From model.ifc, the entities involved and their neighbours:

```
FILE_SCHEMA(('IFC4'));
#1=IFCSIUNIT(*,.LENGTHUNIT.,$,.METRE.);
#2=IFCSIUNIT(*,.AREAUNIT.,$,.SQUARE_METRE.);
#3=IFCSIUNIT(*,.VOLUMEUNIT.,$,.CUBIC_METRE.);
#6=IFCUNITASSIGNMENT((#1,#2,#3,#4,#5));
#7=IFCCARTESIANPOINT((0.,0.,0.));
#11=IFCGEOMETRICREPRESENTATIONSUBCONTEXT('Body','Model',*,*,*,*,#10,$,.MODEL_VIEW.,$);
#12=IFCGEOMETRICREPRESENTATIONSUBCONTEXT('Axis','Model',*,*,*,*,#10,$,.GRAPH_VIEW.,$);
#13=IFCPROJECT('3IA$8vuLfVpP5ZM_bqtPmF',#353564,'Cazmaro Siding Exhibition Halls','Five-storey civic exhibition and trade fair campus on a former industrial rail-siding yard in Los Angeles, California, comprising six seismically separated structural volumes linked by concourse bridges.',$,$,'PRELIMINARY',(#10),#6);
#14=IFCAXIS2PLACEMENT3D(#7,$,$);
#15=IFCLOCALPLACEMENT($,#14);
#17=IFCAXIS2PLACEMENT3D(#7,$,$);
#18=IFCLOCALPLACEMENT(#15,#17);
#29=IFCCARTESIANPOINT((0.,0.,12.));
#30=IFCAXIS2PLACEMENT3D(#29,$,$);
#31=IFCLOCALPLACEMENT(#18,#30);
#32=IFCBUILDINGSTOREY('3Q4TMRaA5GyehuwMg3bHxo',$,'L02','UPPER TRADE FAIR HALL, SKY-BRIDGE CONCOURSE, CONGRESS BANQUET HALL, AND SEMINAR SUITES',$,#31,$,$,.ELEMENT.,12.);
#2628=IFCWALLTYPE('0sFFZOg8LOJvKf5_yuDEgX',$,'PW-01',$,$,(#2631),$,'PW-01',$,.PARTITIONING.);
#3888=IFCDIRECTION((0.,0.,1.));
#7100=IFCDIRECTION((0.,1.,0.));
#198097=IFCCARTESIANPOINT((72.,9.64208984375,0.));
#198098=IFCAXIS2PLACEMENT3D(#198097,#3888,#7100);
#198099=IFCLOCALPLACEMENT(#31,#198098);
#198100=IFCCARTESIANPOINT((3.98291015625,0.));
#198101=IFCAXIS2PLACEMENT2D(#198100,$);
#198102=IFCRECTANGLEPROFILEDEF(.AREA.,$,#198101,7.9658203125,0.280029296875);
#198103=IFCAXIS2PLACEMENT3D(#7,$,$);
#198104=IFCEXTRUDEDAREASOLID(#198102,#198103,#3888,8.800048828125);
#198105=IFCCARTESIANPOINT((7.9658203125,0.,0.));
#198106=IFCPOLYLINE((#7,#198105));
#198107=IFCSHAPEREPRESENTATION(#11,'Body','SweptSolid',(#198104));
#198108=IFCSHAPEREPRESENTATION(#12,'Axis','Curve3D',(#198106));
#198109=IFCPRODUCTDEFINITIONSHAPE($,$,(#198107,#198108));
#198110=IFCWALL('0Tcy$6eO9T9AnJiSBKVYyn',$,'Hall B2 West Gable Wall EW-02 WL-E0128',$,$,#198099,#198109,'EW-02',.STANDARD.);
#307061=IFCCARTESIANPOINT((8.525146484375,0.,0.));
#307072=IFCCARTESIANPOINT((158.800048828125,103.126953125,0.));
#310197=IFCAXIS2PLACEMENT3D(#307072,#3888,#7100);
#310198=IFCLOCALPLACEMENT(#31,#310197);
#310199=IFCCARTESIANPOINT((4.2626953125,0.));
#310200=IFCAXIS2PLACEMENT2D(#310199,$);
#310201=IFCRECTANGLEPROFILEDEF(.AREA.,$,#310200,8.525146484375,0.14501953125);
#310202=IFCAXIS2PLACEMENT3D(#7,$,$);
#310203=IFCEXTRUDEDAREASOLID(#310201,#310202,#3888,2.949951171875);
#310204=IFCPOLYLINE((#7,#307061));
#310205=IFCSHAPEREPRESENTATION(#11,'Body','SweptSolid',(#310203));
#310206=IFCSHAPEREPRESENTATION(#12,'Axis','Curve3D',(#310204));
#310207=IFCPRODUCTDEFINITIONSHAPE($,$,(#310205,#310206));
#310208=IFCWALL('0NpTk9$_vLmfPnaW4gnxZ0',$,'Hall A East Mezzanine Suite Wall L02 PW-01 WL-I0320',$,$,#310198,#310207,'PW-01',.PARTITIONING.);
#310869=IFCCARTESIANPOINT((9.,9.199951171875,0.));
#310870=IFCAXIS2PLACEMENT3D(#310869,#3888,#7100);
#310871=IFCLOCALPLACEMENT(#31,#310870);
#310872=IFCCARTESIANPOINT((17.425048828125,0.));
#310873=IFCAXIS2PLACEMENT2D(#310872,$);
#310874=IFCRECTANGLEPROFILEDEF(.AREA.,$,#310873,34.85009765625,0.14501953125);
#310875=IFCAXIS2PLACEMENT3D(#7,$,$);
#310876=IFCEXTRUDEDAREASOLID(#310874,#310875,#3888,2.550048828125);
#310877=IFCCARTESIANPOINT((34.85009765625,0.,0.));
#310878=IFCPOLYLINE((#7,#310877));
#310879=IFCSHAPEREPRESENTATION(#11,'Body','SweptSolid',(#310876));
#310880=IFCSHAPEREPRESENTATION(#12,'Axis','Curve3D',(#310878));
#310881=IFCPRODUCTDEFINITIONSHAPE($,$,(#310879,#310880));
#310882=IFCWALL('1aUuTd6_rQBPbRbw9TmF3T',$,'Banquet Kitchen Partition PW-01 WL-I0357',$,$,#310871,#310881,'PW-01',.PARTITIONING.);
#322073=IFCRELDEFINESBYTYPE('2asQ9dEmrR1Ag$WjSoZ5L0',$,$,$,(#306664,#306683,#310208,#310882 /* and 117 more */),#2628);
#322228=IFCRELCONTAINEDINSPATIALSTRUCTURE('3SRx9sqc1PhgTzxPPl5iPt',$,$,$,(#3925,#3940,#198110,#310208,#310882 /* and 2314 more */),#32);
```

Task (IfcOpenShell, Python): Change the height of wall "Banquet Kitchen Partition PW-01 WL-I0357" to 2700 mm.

```python
import ifcopenshell
import ifcopenshell.geom
import ifcopenshell.util.representation
import ifcopenshell.util.shape
import ifcopenshell.util.unit

model = ifcopenshell.open("model.ifc")
unit_scale = ifcopenshell.util.unit.calculate_unit_scale(model)
settings = ifcopenshell.geom.settings()


def volume(element):
    """Net volume in cubic metres, openings subtracted."""
    shape = ifcopenshell.geom.create_shape(settings, element)
    return ifcopenshell.util.shape.get_volume(shape.geometry)


wall = model.by_guid("1aUuTd6_rQBPbRbw9TmF3T")
before = volume(wall)

body = ifcopenshell.util.representation.get_representation(wall, "Model", "Body")
solid = body.Items[0]
old_height = solid.Depth
solid.Depth = 2.7 / unit_scale
after = volume(wall)

print(f"height {old_height:g} -> {solid.Depth:g}, volume {before:.3f} -> {after:.3f} m3")

model.write("model_v2.ifc")
```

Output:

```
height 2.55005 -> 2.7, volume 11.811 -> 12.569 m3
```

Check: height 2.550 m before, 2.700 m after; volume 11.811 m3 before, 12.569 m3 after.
